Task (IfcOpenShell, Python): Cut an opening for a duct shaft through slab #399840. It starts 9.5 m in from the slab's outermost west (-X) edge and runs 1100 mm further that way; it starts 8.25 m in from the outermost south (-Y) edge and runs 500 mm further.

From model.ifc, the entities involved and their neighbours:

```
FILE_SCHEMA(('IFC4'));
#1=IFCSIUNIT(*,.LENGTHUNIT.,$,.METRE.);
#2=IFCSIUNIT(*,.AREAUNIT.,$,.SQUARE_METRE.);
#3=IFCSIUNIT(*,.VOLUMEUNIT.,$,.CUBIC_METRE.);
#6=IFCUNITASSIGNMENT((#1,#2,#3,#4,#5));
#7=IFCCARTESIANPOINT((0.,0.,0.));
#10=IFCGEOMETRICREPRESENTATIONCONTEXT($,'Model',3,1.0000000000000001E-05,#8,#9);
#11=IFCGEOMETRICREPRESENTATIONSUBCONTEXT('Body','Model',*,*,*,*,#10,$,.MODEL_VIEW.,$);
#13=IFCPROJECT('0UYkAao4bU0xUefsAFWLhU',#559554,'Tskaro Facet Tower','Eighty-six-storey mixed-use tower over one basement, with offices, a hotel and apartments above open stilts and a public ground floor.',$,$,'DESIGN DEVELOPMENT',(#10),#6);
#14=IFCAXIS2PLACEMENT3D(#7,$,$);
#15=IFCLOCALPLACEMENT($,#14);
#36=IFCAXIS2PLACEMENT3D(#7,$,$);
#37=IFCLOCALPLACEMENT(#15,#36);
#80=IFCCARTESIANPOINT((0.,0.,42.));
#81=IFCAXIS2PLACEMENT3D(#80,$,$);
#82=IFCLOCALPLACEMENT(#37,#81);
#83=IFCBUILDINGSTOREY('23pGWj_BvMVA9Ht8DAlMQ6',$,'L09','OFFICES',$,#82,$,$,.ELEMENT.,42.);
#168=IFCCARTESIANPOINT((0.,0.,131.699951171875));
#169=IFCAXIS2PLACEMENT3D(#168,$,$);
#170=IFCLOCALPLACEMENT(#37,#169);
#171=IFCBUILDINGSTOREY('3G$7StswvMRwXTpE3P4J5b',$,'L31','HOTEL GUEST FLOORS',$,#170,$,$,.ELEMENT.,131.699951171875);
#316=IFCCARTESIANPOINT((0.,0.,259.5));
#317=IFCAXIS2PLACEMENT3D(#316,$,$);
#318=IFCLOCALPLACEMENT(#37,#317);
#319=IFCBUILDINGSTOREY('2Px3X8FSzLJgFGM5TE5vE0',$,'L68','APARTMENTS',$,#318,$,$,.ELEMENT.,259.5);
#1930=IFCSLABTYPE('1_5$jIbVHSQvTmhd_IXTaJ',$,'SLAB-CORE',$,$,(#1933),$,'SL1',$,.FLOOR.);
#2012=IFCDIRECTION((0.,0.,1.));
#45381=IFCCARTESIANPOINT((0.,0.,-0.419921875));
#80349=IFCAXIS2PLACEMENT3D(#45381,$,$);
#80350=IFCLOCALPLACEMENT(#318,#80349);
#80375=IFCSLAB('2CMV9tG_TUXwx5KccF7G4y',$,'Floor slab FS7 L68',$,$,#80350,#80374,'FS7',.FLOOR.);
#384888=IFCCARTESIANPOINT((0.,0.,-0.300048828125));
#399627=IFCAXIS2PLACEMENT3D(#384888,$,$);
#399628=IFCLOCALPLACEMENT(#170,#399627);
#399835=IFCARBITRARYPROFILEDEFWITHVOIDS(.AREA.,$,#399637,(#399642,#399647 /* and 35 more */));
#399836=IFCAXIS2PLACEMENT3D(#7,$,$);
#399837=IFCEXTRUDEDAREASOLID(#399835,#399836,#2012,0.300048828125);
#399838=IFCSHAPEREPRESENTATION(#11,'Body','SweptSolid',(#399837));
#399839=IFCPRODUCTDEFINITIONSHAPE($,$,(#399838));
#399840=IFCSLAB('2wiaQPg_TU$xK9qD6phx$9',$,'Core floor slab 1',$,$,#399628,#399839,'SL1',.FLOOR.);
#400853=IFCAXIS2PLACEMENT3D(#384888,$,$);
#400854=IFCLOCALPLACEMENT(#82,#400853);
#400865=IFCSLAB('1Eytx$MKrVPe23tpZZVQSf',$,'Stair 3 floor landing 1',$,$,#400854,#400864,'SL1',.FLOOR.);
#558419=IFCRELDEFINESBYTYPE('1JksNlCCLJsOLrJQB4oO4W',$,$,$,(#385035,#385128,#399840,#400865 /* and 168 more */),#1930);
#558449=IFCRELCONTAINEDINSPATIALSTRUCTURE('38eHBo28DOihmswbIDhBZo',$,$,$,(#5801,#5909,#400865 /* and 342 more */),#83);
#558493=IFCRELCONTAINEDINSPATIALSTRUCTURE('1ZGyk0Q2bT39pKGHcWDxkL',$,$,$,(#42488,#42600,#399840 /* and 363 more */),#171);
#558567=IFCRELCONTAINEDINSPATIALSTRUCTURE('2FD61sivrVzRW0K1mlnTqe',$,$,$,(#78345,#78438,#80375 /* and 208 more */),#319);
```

```python
import numpy as np
import ifcopenshell
import ifcopenshell.api.feature
import ifcopenshell.api.geometry
import ifcopenshell.api.root
import ifcopenshell.geom
import ifcopenshell.util.placement
import ifcopenshell.util.representation
import ifcopenshell.util.shape
import ifcopenshell.util.unit

model = ifcopenshell.open("model.ifc")
unit_scale = ifcopenshell.util.unit.calculate_unit_scale(model)
settings = ifcopenshell.geom.settings()


def volume(element):
    """Net volume in cubic metres, openings subtracted."""
    shape = ifcopenshell.geom.create_shape(settings, element)
    return ifcopenshell.util.shape.get_volume(shape.geometry)


slab = model.by_guid("2wiaQPg_TU$xK9qD6phx$9")
before = volume(slab)

# Extent in the slab's own axes, in metres. The edges named are its -X and -Y sides.
slab_shape = ifcopenshell.geom.create_shape(settings, slab)
vertices = ifcopenshell.util.shape.get_vertices(slab_shape.geometry)
x_min, y_min, bottom = vertices.min(axis=0)
top = vertices[:, 2].max()

opening = ifcopenshell.api.root.create_entity(model, ifc_class="IfcOpeningElement", name="Duct shaft opening", predefined_type="OPENING")
context = ifcopenshell.util.representation.get_context(model, "Model", "Body", "MODEL_VIEW")
width, depth = 1.1, 0.5
outline = [(0.0, 0.0), (width, 0.0), (width, depth), (0.0, depth), (0.0, 0.0)]
# Overshoot both faces by 50 mm so the cut is clean.
shape = ifcopenshell.api.geometry.add_slab_representation(
    model, context=context, depth=top - bottom + 0.1, polyline=outline
)
ifcopenshell.api.geometry.assign_representation(model, product=opening, representation=shape)

matrix = ifcopenshell.util.placement.get_local_placement(slab.ObjectPlacement)
matrix[:, 3] = matrix @ np.append(np.array([x_min + 9.5, y_min + 8.25, bottom - 0.05]) / unit_scale, 1.0)
ifcopenshell.api.geometry.edit_object_placement(model, product=opening, matrix=matrix, is_si=False)
ifcopenshell.api.feature.add_feature(model, feature=opening, element=slab)

after = volume(slab)

print(f"slab volume {before:.3f} -> {after:.3f} m3")

model.write("model_v2.ifc")
```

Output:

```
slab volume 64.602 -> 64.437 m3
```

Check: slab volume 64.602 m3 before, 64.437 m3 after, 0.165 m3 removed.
